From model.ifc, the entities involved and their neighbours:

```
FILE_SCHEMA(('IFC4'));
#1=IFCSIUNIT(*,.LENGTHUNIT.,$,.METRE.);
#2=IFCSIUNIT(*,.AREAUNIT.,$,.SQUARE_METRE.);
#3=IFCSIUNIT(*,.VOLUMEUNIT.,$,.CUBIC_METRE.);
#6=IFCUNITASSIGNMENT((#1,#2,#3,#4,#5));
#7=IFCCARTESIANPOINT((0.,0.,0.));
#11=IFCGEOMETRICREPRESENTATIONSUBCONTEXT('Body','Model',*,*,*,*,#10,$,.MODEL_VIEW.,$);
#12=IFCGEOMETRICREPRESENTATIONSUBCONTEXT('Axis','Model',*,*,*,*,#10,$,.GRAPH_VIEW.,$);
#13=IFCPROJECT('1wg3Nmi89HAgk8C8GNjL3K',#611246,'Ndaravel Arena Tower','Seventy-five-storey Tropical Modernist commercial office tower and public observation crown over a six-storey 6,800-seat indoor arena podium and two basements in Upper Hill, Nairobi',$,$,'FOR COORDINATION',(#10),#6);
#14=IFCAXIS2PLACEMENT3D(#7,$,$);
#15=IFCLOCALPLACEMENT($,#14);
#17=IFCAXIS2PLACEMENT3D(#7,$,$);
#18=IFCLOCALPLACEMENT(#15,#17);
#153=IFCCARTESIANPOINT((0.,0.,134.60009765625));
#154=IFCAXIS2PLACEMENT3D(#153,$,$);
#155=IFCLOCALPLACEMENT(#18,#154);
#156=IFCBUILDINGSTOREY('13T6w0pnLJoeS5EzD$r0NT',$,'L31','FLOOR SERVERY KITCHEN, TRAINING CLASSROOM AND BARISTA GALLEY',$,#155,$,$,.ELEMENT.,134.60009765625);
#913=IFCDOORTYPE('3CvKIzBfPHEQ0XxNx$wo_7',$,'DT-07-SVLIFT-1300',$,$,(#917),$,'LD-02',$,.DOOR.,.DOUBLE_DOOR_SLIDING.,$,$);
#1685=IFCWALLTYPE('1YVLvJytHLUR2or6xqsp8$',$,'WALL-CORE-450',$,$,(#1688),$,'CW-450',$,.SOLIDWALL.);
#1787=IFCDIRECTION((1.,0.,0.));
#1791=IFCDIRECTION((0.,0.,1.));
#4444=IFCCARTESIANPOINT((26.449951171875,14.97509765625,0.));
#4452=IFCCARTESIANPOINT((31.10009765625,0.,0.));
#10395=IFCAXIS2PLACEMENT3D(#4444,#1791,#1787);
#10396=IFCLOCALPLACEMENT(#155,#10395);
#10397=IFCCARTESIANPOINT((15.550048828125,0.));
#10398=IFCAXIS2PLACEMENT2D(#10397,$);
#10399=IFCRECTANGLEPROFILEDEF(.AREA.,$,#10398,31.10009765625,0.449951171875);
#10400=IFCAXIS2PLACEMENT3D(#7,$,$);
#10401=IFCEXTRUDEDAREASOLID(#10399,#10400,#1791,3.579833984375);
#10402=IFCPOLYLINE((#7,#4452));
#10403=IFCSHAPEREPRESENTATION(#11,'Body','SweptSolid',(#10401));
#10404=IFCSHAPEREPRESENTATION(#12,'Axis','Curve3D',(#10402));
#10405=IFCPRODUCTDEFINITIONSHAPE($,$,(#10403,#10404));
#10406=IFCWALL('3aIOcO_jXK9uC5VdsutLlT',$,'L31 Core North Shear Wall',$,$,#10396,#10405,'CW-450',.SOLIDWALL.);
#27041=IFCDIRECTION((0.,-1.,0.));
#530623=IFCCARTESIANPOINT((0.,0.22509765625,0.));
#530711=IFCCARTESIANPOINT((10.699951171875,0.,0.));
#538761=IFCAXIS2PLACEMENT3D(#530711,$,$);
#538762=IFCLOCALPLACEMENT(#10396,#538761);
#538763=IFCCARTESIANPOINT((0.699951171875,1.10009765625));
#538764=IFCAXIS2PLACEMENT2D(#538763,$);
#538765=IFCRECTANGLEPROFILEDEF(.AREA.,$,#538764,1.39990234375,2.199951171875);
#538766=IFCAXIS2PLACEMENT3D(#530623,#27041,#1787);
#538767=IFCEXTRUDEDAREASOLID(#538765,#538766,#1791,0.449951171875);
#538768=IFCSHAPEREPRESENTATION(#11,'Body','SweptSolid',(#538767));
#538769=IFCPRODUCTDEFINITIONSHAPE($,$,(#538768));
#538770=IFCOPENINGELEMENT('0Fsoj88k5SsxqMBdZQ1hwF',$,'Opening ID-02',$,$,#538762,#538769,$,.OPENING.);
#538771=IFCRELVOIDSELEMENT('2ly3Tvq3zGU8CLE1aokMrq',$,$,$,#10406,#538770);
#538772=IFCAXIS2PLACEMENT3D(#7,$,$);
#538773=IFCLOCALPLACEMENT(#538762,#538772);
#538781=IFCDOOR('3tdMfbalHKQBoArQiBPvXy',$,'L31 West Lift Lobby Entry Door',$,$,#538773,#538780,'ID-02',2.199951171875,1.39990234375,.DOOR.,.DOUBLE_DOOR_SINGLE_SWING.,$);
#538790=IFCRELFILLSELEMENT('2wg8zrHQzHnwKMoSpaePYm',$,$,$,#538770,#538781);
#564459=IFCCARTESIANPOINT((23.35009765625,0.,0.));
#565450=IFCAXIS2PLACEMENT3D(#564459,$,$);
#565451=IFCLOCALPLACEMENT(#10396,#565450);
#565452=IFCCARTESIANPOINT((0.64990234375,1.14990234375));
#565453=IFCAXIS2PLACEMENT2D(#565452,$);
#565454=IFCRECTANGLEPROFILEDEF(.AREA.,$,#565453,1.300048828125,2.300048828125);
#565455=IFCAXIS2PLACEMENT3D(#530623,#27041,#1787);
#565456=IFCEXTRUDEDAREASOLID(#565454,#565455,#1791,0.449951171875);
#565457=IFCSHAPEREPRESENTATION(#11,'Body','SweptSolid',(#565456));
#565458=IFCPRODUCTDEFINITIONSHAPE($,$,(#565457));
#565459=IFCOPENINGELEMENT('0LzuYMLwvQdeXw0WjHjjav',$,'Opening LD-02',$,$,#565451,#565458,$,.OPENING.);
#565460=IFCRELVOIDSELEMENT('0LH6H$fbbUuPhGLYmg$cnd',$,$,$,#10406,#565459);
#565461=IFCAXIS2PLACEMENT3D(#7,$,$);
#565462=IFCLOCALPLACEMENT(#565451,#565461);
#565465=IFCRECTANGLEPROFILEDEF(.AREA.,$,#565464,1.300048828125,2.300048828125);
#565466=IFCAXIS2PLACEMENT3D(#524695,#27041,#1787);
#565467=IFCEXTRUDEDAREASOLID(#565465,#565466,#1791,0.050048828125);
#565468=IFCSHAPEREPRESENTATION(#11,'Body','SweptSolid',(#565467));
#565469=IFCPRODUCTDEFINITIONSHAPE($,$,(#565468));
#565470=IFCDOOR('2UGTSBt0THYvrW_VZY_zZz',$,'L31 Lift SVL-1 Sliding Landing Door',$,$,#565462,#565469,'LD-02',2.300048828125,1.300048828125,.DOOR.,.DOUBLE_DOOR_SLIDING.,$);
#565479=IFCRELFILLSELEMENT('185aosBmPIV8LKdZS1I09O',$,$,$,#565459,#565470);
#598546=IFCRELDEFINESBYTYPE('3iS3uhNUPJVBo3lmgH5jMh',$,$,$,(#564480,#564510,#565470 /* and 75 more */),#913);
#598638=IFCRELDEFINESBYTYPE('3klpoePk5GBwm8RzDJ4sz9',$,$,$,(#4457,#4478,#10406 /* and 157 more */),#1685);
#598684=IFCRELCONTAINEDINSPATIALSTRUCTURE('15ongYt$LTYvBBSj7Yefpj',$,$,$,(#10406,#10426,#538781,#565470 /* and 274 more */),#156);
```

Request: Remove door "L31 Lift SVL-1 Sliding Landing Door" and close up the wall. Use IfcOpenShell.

```python
import ifcopenshell
import ifcopenshell.api.feature
import ifcopenshell.api.root
import ifcopenshell.geom
import ifcopenshell.util.shape

model = ifcopenshell.open("model.ifc")
settings = ifcopenshell.geom.settings()


def volume(element):
    """Net volume in cubic metres, openings subtracted."""
    shape = ifcopenshell.geom.create_shape(settings, element)
    return ifcopenshell.util.shape.get_volume(shape.geometry)


door = model.by_id(565470)
opening = door.FillsVoids[0].RelatingOpeningElement
wall = opening.VoidsElements[0].RelatingBuildingElement
before = volume(wall)

ifcopenshell.api.root.remove_product(model, product=door)
ifcopenshell.api.feature.remove_feature(model, feature=opening)

after = volume(wall)

print(f"wall volume {before:.3f} -> {after:.3f} m3")

model.write("model-out.ifc")
```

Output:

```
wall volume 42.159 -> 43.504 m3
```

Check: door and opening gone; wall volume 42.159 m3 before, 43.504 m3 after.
